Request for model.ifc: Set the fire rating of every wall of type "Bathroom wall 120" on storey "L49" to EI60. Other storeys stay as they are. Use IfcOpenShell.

First a look at what the model holds.

```python
import ifcopenshell
import ifcopenshell.util.element

model = ifcopenshell.open("model.ifc")
print(model.schema)
storey = next(s for s in model.by_type("IfcBuildingStorey") if s.Name == "L49")
walls = [e for e in ifcopenshell.util.element.get_decomposition(storey) if e.is_a("IfcWall")]
seen = {}
for e in walls:
    element_type = ifcopenshell.util.element.get_type(e)
    key = (element_type.Name if element_type != e and element_type else None, ifcopenshell.util.element.get_pset(e, "Pset_WallCommon", "FireRating"))
    seen[key] = seen.get(key, 0) + 1
for (name, value), count in sorted(seen.items(), key=str):
    print(count, "x", name, "|", value)
```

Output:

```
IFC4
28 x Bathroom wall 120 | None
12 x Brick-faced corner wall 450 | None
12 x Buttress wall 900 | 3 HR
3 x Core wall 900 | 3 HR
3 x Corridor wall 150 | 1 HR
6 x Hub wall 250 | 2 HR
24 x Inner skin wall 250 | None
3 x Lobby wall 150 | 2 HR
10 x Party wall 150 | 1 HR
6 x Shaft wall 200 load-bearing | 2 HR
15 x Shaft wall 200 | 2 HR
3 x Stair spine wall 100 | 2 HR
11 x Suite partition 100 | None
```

```python
import ifcopenshell
import ifcopenshell.api.pset
import ifcopenshell.util.element

model = ifcopenshell.open("model.ifc")

storey = next(s for s in model.by_type("IfcBuildingStorey") if s.Name == "L49")
walls = [e for e in ifcopenshell.util.element.get_decomposition(storey) if e.is_a("IfcWall")]

count = 0
for e in walls:
    element_type = ifcopenshell.util.element.get_type(e)
    if element_type in (None, e) or element_type.Name != "Bathroom wall 120":
        continue
    found = ifcopenshell.util.element.get_pset(e, "Pset_WallCommon", should_inherit=False)
    if found:
        pset = model.by_id(found["id"])
        if len(ifcopenshell.util.element.get_elements_by_pset(pset)) > 1:
            pset = ifcopenshell.api.pset.unshare_pset(model, products=[e], pset=pset)[0]
    else:
        pset = ifcopenshell.api.pset.add_pset(model, product=e, name="Pset_WallCommon")
    ifcopenshell.api.pset.edit_pset(model, pset=pset, properties={"FireRating": "EI60"})
    count += 1

print(count, "walls updated")

model.write("model_edited.ifc")
```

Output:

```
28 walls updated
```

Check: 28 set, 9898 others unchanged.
